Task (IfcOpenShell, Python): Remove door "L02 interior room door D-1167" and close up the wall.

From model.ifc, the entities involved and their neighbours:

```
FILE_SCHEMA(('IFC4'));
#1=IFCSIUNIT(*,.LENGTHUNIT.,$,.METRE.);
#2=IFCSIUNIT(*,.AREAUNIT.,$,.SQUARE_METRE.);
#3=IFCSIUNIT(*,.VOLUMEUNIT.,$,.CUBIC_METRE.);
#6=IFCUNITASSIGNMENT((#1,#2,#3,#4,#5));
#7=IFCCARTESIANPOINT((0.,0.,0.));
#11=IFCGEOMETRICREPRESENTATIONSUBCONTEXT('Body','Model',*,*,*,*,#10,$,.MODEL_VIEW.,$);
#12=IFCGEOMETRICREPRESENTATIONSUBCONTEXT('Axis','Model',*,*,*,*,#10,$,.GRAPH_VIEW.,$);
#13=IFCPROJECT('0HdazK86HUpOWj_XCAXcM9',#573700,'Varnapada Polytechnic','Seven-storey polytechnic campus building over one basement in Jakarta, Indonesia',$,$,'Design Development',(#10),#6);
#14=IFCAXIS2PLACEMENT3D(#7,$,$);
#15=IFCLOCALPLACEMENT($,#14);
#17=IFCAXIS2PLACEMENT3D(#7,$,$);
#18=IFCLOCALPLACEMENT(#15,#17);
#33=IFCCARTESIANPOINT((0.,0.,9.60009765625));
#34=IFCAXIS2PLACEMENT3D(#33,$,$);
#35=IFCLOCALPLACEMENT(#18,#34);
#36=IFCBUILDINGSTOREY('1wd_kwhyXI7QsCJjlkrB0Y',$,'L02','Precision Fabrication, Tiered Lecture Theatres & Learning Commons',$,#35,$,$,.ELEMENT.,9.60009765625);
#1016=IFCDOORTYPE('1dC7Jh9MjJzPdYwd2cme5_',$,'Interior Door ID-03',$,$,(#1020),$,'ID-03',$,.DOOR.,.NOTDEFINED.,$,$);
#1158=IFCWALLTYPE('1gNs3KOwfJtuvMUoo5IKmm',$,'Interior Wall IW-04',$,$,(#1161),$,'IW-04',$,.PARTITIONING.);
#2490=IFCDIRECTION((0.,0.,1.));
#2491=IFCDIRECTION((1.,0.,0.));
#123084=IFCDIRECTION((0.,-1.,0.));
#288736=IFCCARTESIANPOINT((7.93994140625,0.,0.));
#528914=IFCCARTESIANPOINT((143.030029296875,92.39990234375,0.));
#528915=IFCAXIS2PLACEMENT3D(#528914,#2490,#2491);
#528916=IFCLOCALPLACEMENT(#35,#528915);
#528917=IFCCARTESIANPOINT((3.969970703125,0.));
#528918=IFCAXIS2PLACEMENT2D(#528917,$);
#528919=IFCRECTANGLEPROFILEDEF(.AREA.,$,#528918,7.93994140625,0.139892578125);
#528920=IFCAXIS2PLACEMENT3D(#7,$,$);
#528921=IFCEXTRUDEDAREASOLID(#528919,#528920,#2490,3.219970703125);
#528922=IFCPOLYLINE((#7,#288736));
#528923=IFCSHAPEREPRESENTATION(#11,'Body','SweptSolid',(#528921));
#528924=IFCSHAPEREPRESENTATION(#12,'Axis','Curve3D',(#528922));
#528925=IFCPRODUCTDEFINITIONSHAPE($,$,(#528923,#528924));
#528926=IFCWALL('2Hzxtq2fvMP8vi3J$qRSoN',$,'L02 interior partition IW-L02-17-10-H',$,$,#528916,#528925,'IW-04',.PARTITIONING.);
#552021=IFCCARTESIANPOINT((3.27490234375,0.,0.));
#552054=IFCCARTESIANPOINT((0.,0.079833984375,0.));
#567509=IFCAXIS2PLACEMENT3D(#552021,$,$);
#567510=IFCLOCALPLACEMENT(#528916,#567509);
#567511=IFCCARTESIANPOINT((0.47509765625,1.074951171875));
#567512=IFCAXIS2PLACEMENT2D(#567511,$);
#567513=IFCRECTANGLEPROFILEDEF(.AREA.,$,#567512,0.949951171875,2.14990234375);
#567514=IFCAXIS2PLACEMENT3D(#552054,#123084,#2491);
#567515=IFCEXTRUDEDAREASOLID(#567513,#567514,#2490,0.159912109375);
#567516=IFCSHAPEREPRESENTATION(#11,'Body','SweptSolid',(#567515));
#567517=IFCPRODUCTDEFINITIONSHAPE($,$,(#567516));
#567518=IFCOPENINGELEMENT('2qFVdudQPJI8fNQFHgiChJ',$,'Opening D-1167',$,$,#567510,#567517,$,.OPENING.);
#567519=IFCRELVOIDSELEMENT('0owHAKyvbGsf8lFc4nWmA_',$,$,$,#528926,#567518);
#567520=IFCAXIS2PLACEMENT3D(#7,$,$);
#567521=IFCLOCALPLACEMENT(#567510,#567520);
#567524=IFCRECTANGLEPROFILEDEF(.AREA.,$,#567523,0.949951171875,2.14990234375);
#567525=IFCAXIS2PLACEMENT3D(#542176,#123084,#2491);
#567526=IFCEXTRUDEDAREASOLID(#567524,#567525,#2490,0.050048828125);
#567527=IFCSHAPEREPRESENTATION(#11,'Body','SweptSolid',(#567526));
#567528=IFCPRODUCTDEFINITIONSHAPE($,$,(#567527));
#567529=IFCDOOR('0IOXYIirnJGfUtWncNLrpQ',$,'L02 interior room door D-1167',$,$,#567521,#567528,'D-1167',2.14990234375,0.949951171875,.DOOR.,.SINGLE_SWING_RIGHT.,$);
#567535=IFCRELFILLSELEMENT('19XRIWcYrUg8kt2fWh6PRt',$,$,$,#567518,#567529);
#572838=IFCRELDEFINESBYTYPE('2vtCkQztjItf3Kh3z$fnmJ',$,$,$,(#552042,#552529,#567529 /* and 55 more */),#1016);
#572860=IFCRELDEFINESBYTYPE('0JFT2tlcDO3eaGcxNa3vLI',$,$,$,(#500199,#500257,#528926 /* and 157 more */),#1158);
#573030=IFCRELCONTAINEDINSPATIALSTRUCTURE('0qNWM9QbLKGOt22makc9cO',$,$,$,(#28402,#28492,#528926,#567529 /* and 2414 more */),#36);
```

```python
import ifcopenshell
import ifcopenshell.api.feature
import ifcopenshell.api.root
import ifcopenshell.geom
import ifcopenshell.util.shape

model = ifcopenshell.open("model.ifc")
settings = ifcopenshell.geom.settings()


def volume(element):
    """Net volume in cubic metres, openings subtracted."""
    shape = ifcopenshell.geom.create_shape(settings, element)
    return ifcopenshell.util.shape.get_volume(shape.geometry)


door = model.by_id(567529)
opening = door.FillsVoids[0].RelatingOpeningElement
wall = opening.VoidsElements[0].RelatingBuildingElement
before = volume(wall)

ifcopenshell.api.root.remove_product(model, product=door)
ifcopenshell.api.feature.remove_feature(model, feature=opening)

after = volume(wall)

print(f"wall volume {before:.3f} -> {after:.3f} m3")

model.write("model_v2.ifc")
```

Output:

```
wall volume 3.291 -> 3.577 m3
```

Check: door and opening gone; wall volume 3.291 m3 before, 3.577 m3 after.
